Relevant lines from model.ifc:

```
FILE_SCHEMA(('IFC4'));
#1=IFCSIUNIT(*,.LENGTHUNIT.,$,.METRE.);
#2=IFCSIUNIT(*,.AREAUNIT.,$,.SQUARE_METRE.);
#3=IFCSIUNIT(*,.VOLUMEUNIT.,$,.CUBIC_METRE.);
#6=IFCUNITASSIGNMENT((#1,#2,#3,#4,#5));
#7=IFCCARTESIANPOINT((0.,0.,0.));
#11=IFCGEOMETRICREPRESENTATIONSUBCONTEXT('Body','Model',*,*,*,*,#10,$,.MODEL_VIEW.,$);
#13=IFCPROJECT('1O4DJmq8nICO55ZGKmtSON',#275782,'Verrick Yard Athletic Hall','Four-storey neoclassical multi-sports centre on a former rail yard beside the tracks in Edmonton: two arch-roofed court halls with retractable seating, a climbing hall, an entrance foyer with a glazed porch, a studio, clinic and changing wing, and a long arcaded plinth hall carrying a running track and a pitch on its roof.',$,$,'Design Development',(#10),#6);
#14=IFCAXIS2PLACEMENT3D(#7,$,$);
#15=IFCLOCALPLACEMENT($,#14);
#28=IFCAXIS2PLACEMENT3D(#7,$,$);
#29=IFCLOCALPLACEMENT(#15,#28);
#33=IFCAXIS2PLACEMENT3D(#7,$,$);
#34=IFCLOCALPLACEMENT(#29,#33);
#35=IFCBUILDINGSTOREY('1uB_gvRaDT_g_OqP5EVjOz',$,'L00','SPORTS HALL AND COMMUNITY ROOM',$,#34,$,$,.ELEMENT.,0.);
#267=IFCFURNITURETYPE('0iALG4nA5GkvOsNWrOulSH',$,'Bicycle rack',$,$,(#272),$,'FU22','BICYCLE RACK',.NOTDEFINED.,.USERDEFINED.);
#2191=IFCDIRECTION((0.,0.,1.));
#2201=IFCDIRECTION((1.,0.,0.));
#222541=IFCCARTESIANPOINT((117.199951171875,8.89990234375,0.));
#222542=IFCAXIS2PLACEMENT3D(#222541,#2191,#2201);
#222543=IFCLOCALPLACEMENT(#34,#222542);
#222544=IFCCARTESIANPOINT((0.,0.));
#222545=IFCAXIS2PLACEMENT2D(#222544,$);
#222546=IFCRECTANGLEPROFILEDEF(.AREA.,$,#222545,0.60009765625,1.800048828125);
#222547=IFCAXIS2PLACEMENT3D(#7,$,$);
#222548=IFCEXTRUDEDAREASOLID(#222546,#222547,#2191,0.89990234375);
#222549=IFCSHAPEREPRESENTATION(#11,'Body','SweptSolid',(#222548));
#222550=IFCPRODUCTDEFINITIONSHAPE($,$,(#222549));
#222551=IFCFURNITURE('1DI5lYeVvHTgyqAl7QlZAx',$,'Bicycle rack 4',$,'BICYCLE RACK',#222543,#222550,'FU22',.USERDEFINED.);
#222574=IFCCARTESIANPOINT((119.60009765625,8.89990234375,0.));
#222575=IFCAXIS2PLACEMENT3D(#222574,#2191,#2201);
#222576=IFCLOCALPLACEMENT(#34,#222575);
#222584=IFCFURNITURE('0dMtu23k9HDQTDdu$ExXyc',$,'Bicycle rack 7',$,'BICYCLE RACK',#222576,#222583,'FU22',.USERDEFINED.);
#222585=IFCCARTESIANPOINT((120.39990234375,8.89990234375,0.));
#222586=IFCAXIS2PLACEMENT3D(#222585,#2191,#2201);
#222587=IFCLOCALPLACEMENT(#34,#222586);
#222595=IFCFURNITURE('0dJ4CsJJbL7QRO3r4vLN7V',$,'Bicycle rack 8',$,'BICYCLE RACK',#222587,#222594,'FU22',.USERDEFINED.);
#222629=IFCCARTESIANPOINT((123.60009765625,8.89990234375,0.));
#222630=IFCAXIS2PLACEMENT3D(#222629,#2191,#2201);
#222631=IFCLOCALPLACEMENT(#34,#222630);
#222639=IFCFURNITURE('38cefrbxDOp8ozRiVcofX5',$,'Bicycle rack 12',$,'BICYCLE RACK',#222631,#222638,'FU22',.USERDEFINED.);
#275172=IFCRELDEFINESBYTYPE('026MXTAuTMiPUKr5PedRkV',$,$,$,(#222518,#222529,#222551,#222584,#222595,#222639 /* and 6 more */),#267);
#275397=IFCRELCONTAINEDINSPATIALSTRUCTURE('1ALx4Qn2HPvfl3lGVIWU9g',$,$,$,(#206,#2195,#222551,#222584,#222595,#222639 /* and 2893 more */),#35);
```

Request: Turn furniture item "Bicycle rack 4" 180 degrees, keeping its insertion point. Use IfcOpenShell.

```python
import ifcopenshell
import ifcopenshell.api.geometry
import ifcopenshell.util.placement

model = ifcopenshell.open("model.ifc")

item = model.by_guid("1DI5lYeVvHTgyqAl7QlZAx")
matrix = ifcopenshell.util.placement.get_local_placement(item.ObjectPlacement)
matrix = matrix @ ifcopenshell.util.placement.rotation(180, "Z")
ifcopenshell.api.geometry.edit_object_placement(model, product=item, matrix=matrix, is_si=False)

print(ifcopenshell.util.placement.get_local_placement(item.ObjectPlacement).round(3) + 0.0)

model.write("model_v2.ifc")
```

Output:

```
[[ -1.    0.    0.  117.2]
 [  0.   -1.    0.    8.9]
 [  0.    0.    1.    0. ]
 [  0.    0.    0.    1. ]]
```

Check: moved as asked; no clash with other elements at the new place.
